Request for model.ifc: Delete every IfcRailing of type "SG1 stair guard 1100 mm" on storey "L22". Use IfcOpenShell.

First a look at what the model holds.

```python
import ifcopenshell
import ifcopenshell.util.element

model = ifcopenshell.open("model.ifc")
print(model.schema)
storey = next(s for s in model.by_type("IfcBuildingStorey") if s.Name == "L22")
railings = [e for e in ifcopenshell.util.element.get_decomposition(storey) if e.is_a("IfcRailing")]
seen = {}
for e in railings:
    element_type = ifcopenshell.util.element.get_type(e)
    name = element_type.Name if element_type not in (None, e) else None
    seen[name] = seen.get(name, 0) + 1
for name, count in sorted(seen.items(), key=str):
    print(count, "x", name)
```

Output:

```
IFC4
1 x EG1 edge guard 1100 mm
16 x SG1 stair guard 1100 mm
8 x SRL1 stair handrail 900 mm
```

```python
import ifcopenshell
import ifcopenshell.api.root
import ifcopenshell.util.element

model = ifcopenshell.open("model.ifc")

storey = next(s for s in model.by_type("IfcBuildingStorey") if s.Name == "L22")
railings = [e for e in ifcopenshell.util.element.get_decomposition(storey) if e.is_a("IfcRailing")]
targets = [e for e in railings if (t := ifcopenshell.util.element.get_type(e)) not in (None, e) and t.Name == "SG1 stair guard 1100 mm"]

for e in targets:
    ifcopenshell.api.root.remove_product(model, product=e)
print(len(targets), "removed")

model.write("model_v2.ifc")
```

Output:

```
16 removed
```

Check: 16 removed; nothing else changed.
